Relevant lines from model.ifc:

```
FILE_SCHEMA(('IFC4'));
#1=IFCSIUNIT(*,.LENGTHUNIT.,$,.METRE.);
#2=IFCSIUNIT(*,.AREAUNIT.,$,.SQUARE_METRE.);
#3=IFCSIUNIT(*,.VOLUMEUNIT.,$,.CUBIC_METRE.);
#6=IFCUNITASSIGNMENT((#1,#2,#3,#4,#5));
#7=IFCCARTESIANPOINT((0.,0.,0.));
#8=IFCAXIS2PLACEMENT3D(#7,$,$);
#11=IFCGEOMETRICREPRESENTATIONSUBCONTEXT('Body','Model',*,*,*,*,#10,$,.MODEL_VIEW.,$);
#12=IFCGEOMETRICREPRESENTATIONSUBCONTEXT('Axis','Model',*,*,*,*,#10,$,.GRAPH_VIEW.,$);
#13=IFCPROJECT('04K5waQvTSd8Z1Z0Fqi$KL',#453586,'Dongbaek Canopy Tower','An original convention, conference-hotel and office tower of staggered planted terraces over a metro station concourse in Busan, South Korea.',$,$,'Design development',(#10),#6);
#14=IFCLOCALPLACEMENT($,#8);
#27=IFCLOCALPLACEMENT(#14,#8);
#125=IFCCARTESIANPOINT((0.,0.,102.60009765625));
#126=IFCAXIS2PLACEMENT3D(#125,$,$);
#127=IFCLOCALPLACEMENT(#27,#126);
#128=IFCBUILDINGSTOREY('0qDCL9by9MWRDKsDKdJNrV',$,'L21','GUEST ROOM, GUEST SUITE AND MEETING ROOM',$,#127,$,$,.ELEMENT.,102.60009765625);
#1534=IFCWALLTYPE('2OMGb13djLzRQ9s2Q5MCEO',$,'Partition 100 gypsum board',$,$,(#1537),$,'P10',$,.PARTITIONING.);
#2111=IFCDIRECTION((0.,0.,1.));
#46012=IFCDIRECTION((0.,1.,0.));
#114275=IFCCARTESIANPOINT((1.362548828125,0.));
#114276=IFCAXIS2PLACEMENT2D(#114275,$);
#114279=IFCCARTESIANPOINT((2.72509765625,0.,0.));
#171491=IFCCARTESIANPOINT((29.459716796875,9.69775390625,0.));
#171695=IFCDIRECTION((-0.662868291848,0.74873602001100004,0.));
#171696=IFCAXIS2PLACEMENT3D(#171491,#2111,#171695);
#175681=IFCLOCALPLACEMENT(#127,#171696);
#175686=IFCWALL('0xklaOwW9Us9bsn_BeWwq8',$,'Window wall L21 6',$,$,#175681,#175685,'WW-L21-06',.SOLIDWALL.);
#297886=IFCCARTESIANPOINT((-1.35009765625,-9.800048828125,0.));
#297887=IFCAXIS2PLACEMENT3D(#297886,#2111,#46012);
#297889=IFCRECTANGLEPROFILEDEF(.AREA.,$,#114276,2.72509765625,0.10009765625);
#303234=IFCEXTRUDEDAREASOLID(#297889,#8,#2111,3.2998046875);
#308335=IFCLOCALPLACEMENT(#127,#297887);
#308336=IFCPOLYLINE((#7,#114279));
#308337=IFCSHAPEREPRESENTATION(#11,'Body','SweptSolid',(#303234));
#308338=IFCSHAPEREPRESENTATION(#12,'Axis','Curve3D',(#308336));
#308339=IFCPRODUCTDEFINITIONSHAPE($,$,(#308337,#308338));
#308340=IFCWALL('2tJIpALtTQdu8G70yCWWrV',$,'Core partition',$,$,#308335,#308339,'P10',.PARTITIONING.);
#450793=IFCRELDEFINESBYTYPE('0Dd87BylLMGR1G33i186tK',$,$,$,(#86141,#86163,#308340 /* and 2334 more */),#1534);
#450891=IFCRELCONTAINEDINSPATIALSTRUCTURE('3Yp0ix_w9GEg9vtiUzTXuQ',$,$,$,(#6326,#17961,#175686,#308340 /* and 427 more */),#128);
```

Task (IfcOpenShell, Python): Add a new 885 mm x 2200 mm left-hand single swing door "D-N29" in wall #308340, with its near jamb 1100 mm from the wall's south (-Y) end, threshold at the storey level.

```python
import numpy as np
import ifcopenshell
import ifcopenshell.api.feature
import ifcopenshell.api.geometry
import ifcopenshell.api.root
import ifcopenshell.api.spatial
import ifcopenshell.geom
import ifcopenshell.util.element
import ifcopenshell.util.placement
import ifcopenshell.util.representation
import ifcopenshell.util.shape
import ifcopenshell.util.unit

model = ifcopenshell.open("model.ifc")
unit_scale = ifcopenshell.util.unit.calculate_unit_scale(model)
settings = ifcopenshell.geom.settings()


def volume(element):
    """Net volume in cubic metres, openings subtracted."""
    shape = ifcopenshell.geom.create_shape(settings, element)
    return ifcopenshell.util.shape.get_volume(shape.geometry)


wall = model.by_id(308340)
storey = ifcopenshell.util.element.get_container(wall, ifc_class="IfcBuildingStorey")
context = ifcopenshell.util.representation.get_context(model, "Model", "Body", "MODEL_VIEW")
before = volume(wall)

width, height, from_end, sill = 0.885, 2.2, 1.1, 0.0  # metres

# The wall runs along its own X axis, and the end named is its -X end.
wall_shape = ifcopenshell.geom.create_shape(settings, wall)
x, y, z = ifcopenshell.util.shape.get_vertices(wall_shape.geometry).T
start = x.min() + from_end
face, thickness = float(y.min()), float(y.max() - y.min())
wall_matrix = ifcopenshell.util.placement.get_local_placement(wall.ObjectPlacement)
level = ifcopenshell.util.placement.get_local_placement(storey.ObjectPlacement)[2, 3]


def in_wall(x, y):
    """Placement at x, y metres in the wall's axes, at sill height."""
    matrix = wall_matrix.copy()
    matrix[:, 3] = wall_matrix @ np.array([x / unit_scale, y / unit_scale, 0.0, 1.0])
    matrix[2, 3] = level + sill / unit_scale
    return matrix


# Opening: a box that overshoots both wall faces by 50 mm.
opening = ifcopenshell.api.root.create_entity(model, ifc_class="IfcOpeningElement", predefined_type="OPENING")
box = ifcopenshell.api.geometry.add_wall_representation(
    model, context=context, length=width, height=height, thickness=thickness + 0.1
)
ifcopenshell.api.geometry.assign_representation(model, product=opening, representation=box)
ifcopenshell.api.geometry.edit_object_placement(model, product=opening, matrix=in_wall(start, face - 0.05), is_si=False)
ifcopenshell.api.feature.add_feature(model, feature=opening, element=wall)

door = ifcopenshell.api.root.create_entity(model, ifc_class="IfcDoor", name="D-N29", predefined_type="DOOR")
door.OverallWidth, door.OverallHeight = width / unit_scale, height / unit_scale
door.OperationType = "SINGLE_SWING_LEFT"
body = ifcopenshell.api.geometry.add_door_representation(
    model,
    context=context,
    overall_width=door.OverallWidth,
    overall_height=door.OverallHeight,
    operation_type="SINGLE_SWING_LEFT",
    lining_properties={"LiningDepth": thickness / unit_scale, "ThresholdDepth": thickness / unit_scale},
)
ifcopenshell.api.geometry.assign_representation(model, product=door, representation=body)
ifcopenshell.api.spatial.assign_container(model, products=[door], relating_structure=storey)
ifcopenshell.api.feature.add_filling(model, opening=opening, element=door)

# The lining spans the wall, so the door starts at the wall face.
ifcopenshell.api.geometry.edit_object_placement(model, product=door, matrix=in_wall(start, face), is_si=False)

after = volume(wall)

print(f"wall volume {before:.3f} -> {after:.3f} m3")

model.write("model_edited.ifc")
```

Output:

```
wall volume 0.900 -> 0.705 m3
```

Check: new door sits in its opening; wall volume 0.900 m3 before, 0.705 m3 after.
